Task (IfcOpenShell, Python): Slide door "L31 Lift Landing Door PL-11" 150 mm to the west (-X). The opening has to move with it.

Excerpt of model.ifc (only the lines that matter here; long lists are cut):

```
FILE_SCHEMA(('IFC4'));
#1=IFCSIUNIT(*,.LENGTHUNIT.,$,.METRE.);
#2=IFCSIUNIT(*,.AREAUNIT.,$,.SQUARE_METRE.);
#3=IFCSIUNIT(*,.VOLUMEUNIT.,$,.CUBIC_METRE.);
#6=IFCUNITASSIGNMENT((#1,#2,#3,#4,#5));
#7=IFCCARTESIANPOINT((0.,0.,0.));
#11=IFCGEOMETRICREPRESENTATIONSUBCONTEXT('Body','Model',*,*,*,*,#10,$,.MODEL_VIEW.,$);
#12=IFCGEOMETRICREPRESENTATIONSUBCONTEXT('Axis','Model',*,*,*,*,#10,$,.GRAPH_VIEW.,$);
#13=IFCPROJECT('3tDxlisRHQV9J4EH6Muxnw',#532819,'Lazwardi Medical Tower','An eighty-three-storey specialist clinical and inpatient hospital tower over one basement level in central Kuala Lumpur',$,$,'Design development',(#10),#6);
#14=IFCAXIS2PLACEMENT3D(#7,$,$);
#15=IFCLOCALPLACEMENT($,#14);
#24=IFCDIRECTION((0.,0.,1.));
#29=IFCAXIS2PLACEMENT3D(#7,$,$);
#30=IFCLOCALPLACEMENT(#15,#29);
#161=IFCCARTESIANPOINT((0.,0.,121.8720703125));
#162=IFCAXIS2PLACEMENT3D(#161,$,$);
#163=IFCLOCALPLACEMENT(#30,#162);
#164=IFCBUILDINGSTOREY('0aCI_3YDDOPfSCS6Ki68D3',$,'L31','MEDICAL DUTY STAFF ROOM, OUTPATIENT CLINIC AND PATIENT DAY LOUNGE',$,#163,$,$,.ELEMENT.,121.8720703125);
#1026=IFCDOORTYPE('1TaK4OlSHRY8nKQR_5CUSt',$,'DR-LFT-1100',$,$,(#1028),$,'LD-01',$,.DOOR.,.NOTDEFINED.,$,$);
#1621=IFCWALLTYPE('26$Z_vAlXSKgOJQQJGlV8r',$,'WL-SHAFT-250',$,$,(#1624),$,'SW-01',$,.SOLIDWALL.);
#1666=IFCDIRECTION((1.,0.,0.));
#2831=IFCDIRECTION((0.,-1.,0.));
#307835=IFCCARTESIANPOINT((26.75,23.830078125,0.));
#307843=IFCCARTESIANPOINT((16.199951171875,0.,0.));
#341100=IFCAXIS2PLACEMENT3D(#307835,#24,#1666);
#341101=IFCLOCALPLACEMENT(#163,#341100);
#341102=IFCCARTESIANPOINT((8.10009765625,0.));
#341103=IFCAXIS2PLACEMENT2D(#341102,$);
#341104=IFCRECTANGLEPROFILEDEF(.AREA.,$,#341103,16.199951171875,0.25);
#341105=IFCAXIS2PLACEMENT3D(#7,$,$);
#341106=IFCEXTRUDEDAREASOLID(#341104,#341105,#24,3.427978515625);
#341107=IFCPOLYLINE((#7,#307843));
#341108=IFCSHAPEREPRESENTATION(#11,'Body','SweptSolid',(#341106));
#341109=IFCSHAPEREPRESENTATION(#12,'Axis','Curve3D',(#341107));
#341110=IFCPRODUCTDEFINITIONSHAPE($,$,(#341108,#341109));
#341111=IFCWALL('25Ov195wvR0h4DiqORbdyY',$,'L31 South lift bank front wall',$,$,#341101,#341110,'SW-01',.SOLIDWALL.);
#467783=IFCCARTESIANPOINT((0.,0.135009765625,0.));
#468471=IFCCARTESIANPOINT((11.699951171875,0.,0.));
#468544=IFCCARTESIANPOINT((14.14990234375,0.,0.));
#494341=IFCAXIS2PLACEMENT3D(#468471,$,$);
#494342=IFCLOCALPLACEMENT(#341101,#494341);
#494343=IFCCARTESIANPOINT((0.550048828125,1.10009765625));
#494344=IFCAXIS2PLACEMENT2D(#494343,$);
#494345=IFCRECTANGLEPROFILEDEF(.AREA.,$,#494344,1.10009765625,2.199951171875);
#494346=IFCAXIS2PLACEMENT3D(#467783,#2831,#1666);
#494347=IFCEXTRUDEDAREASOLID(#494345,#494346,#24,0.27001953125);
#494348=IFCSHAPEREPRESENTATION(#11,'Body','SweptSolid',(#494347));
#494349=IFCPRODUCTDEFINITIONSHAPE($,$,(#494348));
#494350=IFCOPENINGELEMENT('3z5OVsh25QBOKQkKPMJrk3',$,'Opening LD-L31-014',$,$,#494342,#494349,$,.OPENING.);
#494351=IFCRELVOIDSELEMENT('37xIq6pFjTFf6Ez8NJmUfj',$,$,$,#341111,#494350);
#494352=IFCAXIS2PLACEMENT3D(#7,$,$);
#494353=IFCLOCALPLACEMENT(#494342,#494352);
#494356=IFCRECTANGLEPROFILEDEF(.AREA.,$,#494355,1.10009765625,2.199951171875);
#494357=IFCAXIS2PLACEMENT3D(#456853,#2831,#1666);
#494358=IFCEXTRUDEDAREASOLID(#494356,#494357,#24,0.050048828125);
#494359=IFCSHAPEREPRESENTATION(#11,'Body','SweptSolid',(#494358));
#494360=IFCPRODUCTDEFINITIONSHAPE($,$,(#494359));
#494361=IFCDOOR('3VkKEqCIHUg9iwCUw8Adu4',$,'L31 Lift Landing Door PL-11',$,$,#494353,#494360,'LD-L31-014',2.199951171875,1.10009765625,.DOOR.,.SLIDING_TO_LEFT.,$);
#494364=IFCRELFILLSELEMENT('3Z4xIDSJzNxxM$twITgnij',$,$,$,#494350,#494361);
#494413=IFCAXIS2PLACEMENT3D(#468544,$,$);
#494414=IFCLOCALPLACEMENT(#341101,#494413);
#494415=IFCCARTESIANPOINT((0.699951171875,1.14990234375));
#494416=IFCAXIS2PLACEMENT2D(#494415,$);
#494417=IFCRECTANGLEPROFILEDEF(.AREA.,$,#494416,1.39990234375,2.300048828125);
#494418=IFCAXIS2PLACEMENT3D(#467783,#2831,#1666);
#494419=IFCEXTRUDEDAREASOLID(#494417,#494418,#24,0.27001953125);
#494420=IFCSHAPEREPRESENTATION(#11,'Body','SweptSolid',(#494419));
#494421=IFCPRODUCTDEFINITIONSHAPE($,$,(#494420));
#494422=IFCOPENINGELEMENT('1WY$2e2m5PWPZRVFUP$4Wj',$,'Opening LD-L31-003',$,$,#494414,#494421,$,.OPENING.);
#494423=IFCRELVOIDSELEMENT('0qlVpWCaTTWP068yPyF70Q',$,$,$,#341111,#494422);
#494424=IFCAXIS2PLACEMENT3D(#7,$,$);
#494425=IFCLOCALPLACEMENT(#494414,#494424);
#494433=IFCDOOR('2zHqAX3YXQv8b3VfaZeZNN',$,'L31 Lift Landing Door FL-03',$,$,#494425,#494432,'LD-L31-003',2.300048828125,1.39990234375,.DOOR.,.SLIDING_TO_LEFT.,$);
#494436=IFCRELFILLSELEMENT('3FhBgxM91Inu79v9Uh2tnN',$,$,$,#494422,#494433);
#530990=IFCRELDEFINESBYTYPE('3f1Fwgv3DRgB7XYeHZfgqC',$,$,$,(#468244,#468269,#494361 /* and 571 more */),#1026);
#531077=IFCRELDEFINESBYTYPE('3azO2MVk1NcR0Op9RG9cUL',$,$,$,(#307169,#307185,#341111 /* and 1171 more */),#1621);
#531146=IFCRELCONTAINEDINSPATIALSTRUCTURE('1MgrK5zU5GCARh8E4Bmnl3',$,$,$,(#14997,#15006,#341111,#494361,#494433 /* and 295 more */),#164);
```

```python
import ifcopenshell
import ifcopenshell.api.geometry
import ifcopenshell.util.placement

model = ifcopenshell.open("model.ifc")

door = model.by_guid("3VkKEqCIHUg9iwCUw8Adu4")
opening = door.FillsVoids[0].RelatingOpeningElement
wall = opening.VoidsElements[0].RelatingBuildingElement

wall_matrix = ifcopenshell.util.placement.get_local_placement(wall.ObjectPlacement)
shift = wall_matrix[:3, 0] * -0.15
before = ifcopenshell.util.placement.get_local_placement(door.ObjectPlacement)[:3, 3].copy()

# The door is placed relative to its opening, so it follows when the opening moves.
matrix = ifcopenshell.util.placement.get_local_placement(opening.ObjectPlacement)
matrix[:3, 3] += shift
ifcopenshell.api.geometry.edit_object_placement(
    model, product=opening, matrix=matrix, is_si=False, should_transform_children=True
)

after = ifcopenshell.util.placement.get_local_placement(door.ObjectPlacement)[:3, 3]
print("door moved by", (after - before).round(3) + 0.0)

model.write("model_v2.ifc")
```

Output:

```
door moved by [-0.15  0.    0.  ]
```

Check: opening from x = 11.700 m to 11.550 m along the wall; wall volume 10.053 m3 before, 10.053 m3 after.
